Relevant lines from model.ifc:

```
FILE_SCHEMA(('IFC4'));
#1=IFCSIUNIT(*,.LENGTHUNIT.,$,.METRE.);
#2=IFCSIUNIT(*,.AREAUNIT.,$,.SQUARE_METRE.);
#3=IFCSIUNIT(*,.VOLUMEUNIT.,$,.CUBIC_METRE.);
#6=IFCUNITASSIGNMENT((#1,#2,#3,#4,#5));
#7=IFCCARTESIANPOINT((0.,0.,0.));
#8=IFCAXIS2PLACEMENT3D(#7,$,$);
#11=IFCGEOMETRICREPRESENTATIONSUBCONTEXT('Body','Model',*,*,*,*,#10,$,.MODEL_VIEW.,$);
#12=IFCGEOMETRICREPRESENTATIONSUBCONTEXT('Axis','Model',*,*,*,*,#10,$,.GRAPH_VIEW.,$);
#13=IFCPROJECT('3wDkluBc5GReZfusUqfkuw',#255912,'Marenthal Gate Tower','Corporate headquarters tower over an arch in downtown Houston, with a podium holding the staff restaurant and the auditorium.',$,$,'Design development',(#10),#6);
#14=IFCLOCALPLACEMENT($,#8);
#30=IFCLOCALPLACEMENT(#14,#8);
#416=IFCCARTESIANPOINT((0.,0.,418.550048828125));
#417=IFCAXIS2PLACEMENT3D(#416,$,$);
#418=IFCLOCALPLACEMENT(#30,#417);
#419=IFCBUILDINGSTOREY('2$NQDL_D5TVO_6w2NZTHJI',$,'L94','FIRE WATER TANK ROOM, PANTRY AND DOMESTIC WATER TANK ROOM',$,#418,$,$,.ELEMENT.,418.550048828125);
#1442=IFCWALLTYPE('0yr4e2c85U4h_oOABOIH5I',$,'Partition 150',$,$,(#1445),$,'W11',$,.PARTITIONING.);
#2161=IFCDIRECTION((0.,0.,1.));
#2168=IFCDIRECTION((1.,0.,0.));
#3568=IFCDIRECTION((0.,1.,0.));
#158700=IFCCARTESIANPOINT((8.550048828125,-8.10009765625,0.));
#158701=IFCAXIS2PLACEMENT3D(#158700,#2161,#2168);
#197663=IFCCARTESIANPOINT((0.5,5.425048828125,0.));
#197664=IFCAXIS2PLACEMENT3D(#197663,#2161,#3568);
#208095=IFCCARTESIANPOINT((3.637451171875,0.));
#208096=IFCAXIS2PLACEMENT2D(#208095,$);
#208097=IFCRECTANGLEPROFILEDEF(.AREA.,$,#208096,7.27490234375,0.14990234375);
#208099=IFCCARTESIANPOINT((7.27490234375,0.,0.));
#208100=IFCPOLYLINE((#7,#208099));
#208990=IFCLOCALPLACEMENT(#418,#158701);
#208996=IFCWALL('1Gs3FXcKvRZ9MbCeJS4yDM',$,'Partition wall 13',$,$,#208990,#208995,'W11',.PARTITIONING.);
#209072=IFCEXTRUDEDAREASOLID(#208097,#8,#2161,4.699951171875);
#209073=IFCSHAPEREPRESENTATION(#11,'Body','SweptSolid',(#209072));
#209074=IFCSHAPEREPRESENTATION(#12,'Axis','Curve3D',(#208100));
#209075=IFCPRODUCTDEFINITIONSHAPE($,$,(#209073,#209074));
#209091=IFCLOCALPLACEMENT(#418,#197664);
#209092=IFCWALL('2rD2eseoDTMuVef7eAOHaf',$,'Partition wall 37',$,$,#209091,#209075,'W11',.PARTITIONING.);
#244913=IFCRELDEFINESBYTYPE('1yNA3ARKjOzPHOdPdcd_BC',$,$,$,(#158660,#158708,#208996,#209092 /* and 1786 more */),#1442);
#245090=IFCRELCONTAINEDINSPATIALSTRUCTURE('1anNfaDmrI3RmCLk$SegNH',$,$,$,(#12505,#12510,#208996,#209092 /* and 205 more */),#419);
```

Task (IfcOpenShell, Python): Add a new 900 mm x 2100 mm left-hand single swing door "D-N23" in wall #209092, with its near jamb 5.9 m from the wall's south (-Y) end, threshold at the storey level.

```python
import numpy as np
import ifcopenshell
import ifcopenshell.api.feature
import ifcopenshell.api.geometry
import ifcopenshell.api.root
import ifcopenshell.api.spatial
import ifcopenshell.geom
import ifcopenshell.util.element
import ifcopenshell.util.placement
import ifcopenshell.util.representation
import ifcopenshell.util.shape
import ifcopenshell.util.unit

model = ifcopenshell.open("model.ifc")
unit_scale = ifcopenshell.util.unit.calculate_unit_scale(model)
settings = ifcopenshell.geom.settings()


def volume(element):
    """Net volume in cubic metres, openings subtracted."""
    shape = ifcopenshell.geom.create_shape(settings, element)
    return ifcopenshell.util.shape.get_volume(shape.geometry)


wall = model.by_id(209092)
storey = ifcopenshell.util.element.get_container(wall, ifc_class="IfcBuildingStorey")
context = ifcopenshell.util.representation.get_context(model, "Model", "Body", "MODEL_VIEW")
before = volume(wall)

width, height, from_end, sill = 0.9, 2.1, 5.9, 0.0  # metres

# The wall runs along its own X axis, and the end named is its -X end.
wall_shape = ifcopenshell.geom.create_shape(settings, wall)
x, y, z = ifcopenshell.util.shape.get_vertices(wall_shape.geometry).T
start = x.min() + from_end
face, thickness = float(y.min()), float(y.max() - y.min())
wall_matrix = ifcopenshell.util.placement.get_local_placement(wall.ObjectPlacement)
level = ifcopenshell.util.placement.get_local_placement(storey.ObjectPlacement)[2, 3]


def in_wall(x, y):
    """Placement at x, y metres in the wall's axes, at sill height."""
    matrix = wall_matrix.copy()
    matrix[:, 3] = wall_matrix @ np.array([x / unit_scale, y / unit_scale, 0.0, 1.0])
    matrix[2, 3] = level + sill / unit_scale
    return matrix


# Opening: a box that overshoots both wall faces by 50 mm.
opening = ifcopenshell.api.root.create_entity(model, ifc_class="IfcOpeningElement", predefined_type="OPENING")
box = ifcopenshell.api.geometry.add_wall_representation(
    model, context=context, length=width, height=height, thickness=thickness + 0.1
)
ifcopenshell.api.geometry.assign_representation(model, product=opening, representation=box)
ifcopenshell.api.geometry.edit_object_placement(model, product=opening, matrix=in_wall(start, face - 0.05), is_si=False)
ifcopenshell.api.feature.add_feature(model, feature=opening, element=wall)

door = ifcopenshell.api.root.create_entity(model, ifc_class="IfcDoor", name="D-N23", predefined_type="DOOR")
door.OverallWidth, door.OverallHeight = width / unit_scale, height / unit_scale
door.OperationType = "SINGLE_SWING_LEFT"
body = ifcopenshell.api.geometry.add_door_representation(
    model,
    context=context,
    overall_width=door.OverallWidth,
    overall_height=door.OverallHeight,
    operation_type="SINGLE_SWING_LEFT",
    lining_properties={"LiningDepth": thickness / unit_scale, "ThresholdDepth": thickness / unit_scale},
)
ifcopenshell.api.geometry.assign_representation(model, product=door, representation=body)
ifcopenshell.api.spatial.assign_container(model, products=[door], relating_structure=storey)
ifcopenshell.api.feature.add_filling(model, opening=opening, element=door)

# The lining spans the wall, so the door starts at the wall face.
ifcopenshell.api.geometry.edit_object_placement(model, product=door, matrix=in_wall(start, face), is_si=False)

after = volume(wall)

print(f"wall volume {before:.3f} -> {after:.3f} m3")

model.write("model_v2.ifc")
```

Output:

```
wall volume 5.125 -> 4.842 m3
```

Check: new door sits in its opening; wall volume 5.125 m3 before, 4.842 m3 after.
